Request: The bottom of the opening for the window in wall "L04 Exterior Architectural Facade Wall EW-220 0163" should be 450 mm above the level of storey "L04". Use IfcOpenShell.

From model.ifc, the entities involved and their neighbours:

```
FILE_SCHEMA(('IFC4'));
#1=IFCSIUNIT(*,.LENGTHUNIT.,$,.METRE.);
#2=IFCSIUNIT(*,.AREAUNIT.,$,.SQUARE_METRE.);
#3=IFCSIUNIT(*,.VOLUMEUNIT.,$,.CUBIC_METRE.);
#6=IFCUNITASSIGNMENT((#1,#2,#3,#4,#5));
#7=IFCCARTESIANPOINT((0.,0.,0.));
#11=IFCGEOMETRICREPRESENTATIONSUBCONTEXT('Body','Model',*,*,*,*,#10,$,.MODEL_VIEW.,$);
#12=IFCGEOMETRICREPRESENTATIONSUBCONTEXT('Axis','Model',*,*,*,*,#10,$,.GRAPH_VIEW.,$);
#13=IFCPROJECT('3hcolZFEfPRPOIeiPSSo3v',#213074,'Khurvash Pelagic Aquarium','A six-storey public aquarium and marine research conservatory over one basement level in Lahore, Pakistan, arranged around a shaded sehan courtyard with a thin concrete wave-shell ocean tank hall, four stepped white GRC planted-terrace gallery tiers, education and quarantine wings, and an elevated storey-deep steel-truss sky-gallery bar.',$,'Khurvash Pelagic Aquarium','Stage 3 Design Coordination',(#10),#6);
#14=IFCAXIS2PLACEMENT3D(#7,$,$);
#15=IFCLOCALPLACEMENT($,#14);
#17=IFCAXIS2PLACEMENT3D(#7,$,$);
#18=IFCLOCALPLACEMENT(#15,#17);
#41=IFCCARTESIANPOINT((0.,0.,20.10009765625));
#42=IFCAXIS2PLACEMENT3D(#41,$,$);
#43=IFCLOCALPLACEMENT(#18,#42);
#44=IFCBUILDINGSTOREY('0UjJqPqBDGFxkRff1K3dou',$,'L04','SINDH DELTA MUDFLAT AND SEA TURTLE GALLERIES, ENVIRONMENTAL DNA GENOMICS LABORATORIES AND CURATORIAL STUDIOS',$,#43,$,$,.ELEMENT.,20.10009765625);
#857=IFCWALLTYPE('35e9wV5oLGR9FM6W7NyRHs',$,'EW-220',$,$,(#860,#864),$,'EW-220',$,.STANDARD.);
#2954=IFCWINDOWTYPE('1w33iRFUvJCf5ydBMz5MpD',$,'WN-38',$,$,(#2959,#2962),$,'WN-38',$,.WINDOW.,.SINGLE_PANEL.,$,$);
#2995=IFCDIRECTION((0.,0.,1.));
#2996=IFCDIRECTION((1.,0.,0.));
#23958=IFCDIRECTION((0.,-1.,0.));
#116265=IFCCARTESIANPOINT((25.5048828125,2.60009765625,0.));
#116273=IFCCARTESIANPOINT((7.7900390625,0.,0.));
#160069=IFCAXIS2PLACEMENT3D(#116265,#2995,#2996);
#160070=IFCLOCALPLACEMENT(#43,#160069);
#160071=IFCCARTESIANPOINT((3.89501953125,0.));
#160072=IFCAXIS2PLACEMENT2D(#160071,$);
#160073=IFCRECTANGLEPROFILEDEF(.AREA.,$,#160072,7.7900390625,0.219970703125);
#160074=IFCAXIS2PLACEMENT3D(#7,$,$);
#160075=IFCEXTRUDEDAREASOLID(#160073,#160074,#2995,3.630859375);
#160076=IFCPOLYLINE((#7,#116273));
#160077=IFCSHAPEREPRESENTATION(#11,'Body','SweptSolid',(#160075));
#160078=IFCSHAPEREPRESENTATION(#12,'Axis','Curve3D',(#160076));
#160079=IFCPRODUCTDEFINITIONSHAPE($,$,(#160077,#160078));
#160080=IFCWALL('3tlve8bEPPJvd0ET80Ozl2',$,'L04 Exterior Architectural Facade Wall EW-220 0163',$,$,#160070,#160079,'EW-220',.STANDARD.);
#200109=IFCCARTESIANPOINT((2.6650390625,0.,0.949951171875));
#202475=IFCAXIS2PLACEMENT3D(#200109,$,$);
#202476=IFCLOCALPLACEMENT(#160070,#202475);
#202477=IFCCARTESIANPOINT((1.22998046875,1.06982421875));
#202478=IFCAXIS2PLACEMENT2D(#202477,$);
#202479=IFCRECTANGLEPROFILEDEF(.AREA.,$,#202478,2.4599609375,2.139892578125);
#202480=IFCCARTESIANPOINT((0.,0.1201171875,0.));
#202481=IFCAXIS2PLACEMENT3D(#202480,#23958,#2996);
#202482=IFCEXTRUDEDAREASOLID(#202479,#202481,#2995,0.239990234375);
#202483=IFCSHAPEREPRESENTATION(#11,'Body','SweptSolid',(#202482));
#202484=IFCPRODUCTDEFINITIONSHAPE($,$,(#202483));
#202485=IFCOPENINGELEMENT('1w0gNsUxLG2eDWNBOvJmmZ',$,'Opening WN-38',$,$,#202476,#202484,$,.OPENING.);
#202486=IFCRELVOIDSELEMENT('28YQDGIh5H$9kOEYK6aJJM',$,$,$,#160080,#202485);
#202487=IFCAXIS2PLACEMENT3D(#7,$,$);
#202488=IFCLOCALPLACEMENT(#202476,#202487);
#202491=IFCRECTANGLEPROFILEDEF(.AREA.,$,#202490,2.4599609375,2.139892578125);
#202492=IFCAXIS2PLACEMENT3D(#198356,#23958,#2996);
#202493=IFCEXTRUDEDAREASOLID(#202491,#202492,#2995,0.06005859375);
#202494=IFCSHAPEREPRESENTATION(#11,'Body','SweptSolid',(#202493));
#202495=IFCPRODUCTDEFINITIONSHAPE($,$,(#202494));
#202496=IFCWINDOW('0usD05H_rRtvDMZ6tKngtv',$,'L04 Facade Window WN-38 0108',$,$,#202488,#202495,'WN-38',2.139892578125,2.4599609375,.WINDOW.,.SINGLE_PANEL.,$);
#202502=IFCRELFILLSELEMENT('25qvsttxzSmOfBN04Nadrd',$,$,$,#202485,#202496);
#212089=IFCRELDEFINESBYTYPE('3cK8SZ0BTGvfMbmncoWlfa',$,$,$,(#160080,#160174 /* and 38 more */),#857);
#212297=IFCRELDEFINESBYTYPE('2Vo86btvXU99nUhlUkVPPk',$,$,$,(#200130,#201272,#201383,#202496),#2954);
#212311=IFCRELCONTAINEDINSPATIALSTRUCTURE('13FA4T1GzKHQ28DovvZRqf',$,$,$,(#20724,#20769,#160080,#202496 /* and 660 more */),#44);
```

```python
import numpy as np
import ifcopenshell
import ifcopenshell.api.geometry
import ifcopenshell.geom
import ifcopenshell.util.element
import ifcopenshell.util.placement
import ifcopenshell.util.shape
import ifcopenshell.util.unit

model = ifcopenshell.open("model.ifc")
unit_scale = ifcopenshell.util.unit.calculate_unit_scale(model)

window = model.by_guid("0usD05H_rRtvDMZ6tKngtv")
opening = window.FillsVoids[0].RelatingOpeningElement
storey = ifcopenshell.util.element.get_container(window, ifc_class="IfcBuildingStorey")
level = ifcopenshell.util.placement.get_local_placement(storey.ObjectPlacement)[2, 3]

# The opening's origin need not be at the sill, so measure its lowest point.
shape = ifcopenshell.geom.create_shape(ifcopenshell.geom.settings(), opening)
bottom = ifcopenshell.util.shape.get_shape_bottom_elevation(shape, shape.geometry) / unit_scale
dz = level + 0.45 - bottom

shift = np.array([0.0, 0.0, dz])
# The window is placed relative to its opening, so it follows when the opening moves.
matrix = ifcopenshell.util.placement.get_local_placement(opening.ObjectPlacement)
matrix[:3, 3] += shift
ifcopenshell.api.geometry.edit_object_placement(
    model, product=opening, matrix=matrix, is_si=False, should_transform_children=True
)

print(f"moved by {dz * unit_scale:+.3f} m")

model.write("model-out.ifc")
```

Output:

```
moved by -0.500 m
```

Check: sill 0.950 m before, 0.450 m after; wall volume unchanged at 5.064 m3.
